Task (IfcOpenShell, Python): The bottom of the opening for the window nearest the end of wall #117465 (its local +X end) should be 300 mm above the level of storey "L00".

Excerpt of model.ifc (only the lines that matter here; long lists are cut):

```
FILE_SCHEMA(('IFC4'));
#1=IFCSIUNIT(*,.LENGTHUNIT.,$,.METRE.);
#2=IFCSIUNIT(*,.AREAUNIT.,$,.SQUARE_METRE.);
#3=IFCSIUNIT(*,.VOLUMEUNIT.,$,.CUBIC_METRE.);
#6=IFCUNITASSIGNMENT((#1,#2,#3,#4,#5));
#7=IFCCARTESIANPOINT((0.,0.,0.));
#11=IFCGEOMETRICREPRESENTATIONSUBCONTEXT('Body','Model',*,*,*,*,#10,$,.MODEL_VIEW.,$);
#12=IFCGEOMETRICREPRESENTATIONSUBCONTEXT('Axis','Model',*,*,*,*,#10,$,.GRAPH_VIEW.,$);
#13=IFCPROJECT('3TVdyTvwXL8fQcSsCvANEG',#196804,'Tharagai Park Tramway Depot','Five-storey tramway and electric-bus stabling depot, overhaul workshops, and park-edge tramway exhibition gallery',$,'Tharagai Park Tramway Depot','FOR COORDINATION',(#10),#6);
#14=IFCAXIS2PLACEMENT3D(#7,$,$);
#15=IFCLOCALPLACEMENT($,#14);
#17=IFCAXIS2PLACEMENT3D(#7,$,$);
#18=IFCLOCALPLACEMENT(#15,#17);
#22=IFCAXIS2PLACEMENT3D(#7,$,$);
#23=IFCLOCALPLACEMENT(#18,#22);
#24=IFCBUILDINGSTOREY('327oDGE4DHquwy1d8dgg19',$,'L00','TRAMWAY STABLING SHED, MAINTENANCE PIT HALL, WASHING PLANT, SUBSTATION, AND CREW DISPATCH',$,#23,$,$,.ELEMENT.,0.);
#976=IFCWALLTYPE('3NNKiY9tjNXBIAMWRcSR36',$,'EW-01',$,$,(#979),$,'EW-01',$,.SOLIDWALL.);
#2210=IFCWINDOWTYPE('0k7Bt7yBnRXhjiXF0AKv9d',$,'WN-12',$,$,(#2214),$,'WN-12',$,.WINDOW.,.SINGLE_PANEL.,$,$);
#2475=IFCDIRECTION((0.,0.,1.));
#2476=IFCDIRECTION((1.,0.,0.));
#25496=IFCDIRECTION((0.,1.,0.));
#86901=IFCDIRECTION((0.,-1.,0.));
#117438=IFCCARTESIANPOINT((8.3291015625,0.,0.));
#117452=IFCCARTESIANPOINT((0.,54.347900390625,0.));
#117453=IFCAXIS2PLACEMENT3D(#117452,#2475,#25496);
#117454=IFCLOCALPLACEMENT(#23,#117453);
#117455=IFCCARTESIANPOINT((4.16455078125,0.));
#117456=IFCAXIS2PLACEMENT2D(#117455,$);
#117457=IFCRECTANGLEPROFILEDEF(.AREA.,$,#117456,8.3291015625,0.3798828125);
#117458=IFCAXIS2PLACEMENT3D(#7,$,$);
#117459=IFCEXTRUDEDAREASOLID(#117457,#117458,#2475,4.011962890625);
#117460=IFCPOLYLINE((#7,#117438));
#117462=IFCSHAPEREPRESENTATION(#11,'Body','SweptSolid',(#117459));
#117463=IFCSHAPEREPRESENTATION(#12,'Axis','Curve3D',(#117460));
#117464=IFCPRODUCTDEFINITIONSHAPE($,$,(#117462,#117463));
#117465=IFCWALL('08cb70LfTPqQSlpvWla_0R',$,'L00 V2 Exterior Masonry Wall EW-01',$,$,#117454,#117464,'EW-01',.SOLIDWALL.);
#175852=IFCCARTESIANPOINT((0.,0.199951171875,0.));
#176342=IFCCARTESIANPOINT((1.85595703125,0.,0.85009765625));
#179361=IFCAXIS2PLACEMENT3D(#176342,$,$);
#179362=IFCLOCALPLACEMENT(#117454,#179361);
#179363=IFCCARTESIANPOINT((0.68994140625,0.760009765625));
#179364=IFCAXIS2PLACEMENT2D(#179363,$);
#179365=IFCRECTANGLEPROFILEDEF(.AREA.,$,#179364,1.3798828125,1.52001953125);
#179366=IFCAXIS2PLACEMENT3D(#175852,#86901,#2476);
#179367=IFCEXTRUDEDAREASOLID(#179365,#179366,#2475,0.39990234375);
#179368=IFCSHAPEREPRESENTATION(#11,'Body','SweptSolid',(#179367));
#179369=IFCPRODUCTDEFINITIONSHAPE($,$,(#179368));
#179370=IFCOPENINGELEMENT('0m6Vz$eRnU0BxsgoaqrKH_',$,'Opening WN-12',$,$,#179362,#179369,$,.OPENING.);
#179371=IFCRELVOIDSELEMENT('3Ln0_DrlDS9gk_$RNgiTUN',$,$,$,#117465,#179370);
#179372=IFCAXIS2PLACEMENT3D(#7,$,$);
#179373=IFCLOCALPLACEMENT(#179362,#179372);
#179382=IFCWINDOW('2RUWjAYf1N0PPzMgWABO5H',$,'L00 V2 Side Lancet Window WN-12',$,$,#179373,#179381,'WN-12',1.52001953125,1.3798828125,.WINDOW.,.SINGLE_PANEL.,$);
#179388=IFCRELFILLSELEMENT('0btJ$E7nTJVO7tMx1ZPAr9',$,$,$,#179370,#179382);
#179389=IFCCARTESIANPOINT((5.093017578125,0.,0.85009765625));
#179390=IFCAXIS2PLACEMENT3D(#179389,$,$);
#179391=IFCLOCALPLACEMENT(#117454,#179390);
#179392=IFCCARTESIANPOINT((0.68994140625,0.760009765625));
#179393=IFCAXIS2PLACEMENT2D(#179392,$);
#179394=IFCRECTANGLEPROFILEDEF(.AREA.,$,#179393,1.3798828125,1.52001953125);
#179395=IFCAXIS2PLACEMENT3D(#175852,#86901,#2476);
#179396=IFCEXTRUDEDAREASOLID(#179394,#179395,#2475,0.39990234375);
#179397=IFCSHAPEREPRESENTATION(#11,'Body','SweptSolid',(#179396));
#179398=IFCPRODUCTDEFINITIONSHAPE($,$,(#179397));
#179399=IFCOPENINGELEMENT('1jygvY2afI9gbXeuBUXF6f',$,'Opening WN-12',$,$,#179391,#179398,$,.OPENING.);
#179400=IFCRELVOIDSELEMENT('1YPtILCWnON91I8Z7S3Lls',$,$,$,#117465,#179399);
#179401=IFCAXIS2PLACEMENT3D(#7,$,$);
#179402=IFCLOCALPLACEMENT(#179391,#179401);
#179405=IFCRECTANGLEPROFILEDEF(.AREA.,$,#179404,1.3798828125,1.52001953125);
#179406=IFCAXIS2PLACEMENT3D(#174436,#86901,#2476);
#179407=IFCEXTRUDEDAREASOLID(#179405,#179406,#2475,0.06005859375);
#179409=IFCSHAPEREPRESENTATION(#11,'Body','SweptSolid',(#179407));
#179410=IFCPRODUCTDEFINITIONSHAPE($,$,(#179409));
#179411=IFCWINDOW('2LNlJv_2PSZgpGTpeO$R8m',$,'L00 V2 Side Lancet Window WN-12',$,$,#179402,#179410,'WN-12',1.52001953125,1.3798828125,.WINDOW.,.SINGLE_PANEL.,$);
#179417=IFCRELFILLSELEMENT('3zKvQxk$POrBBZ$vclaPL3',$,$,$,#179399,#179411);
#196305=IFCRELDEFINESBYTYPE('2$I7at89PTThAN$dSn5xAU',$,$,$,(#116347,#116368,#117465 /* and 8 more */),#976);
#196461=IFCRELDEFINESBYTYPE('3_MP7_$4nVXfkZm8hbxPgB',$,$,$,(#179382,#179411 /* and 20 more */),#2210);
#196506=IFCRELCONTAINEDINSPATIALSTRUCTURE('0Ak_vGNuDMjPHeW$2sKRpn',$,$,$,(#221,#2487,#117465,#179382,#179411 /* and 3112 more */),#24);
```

```python
import numpy as np
import ifcopenshell
import ifcopenshell.api.geometry
import ifcopenshell.geom
import ifcopenshell.util.element
import ifcopenshell.util.placement
import ifcopenshell.util.shape
import ifcopenshell.util.unit

model = ifcopenshell.open("model.ifc")
unit_scale = ifcopenshell.util.unit.calculate_unit_scale(model)

window = model.by_id(179411)
opening = window.FillsVoids[0].RelatingOpeningElement
storey = ifcopenshell.util.element.get_container(window, ifc_class="IfcBuildingStorey")
level = ifcopenshell.util.placement.get_local_placement(storey.ObjectPlacement)[2, 3]

# The opening's origin need not be at the sill, so measure its lowest point.
shape = ifcopenshell.geom.create_shape(ifcopenshell.geom.settings(), opening)
bottom = ifcopenshell.util.shape.get_shape_bottom_elevation(shape, shape.geometry) / unit_scale
dz = level + 0.3 - bottom

shift = np.array([0.0, 0.0, dz])
# The window is placed relative to its opening, so it follows when the opening moves.
matrix = ifcopenshell.util.placement.get_local_placement(opening.ObjectPlacement)
matrix[:3, 3] += shift
ifcopenshell.api.geometry.edit_object_placement(
    model, product=opening, matrix=matrix, is_si=False, should_transform_children=True
)

print(f"moved by {dz * unit_scale:+.3f} m")

model.write("model_rev.ifc")
```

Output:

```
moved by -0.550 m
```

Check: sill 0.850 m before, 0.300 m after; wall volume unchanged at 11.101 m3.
